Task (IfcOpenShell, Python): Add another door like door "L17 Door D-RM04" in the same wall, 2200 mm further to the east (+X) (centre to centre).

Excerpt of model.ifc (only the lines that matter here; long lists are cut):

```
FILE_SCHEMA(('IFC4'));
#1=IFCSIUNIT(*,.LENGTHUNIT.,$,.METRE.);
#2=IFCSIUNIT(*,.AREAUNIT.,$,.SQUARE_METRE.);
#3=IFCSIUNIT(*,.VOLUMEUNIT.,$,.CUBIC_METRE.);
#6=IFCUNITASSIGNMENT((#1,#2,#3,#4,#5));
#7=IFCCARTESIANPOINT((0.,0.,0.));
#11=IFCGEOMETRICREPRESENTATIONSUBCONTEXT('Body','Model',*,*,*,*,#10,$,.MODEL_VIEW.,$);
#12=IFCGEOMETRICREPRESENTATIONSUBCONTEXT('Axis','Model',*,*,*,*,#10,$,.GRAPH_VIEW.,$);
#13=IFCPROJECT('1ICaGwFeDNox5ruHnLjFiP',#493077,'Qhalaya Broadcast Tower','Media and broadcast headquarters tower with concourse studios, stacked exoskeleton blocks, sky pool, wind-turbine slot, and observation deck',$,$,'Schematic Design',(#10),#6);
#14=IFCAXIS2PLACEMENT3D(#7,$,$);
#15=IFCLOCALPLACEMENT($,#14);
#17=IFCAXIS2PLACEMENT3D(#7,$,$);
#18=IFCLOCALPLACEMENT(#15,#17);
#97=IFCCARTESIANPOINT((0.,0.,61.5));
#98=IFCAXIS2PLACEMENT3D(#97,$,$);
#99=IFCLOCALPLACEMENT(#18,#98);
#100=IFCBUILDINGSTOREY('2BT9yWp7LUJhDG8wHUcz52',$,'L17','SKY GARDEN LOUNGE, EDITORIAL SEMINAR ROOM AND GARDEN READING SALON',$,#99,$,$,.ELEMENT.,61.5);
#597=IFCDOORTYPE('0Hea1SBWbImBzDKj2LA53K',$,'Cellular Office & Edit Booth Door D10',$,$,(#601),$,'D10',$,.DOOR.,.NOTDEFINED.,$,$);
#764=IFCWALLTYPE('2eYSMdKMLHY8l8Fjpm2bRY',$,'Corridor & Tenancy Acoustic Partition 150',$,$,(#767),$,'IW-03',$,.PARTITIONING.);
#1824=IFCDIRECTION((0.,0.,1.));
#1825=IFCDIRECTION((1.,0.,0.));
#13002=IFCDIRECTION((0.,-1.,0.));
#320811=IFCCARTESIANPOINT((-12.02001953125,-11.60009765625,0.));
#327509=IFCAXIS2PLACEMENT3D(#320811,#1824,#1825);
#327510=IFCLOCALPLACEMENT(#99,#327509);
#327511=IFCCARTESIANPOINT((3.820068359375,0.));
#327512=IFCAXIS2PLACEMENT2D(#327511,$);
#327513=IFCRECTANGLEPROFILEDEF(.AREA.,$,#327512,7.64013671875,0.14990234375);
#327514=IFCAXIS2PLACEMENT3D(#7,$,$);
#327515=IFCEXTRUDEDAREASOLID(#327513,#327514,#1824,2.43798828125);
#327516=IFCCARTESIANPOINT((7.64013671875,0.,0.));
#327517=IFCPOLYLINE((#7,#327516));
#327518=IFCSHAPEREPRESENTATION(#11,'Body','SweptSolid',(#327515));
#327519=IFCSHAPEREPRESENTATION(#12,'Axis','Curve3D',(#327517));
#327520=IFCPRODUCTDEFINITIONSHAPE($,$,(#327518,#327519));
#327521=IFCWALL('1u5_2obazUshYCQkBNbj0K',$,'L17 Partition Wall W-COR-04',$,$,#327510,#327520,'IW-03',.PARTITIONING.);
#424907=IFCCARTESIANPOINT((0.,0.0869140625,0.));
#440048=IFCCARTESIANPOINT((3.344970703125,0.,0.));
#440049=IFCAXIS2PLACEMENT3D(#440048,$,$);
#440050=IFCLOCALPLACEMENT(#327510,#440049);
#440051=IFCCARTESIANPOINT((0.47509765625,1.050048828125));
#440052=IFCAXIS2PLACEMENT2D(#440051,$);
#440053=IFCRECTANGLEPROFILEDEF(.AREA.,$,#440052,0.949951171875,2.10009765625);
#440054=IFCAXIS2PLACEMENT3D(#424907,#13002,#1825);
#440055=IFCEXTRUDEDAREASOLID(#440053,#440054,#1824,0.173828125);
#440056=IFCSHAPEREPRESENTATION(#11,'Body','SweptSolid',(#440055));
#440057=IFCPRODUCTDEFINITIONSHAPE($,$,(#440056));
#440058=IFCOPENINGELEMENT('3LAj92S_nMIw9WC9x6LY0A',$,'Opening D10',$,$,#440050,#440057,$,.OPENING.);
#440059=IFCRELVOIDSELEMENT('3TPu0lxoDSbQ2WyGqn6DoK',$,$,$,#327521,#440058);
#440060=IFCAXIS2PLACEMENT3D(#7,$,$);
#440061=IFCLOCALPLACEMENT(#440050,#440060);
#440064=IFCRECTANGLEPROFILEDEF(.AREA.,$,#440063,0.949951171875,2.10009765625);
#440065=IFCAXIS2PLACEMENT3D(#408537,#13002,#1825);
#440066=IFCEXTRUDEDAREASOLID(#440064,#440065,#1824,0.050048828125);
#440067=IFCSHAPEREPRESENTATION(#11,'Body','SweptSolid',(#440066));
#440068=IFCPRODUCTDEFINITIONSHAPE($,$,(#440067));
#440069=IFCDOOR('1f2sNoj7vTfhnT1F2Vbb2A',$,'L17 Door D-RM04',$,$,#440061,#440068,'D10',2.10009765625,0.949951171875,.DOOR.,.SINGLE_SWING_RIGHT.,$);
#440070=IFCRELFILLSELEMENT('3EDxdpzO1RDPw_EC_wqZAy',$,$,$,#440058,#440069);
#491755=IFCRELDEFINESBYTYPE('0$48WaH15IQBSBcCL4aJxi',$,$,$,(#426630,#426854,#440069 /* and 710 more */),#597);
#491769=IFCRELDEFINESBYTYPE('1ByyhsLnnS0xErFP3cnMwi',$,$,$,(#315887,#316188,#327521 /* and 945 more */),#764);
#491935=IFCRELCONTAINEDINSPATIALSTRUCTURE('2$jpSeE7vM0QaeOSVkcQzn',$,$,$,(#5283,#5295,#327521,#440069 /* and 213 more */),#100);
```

```python
import ifcopenshell
import ifcopenshell.api.feature
import ifcopenshell.api.geometry
import ifcopenshell.api.root
import ifcopenshell.geom
import ifcopenshell.util.element
import ifcopenshell.util.placement
import ifcopenshell.util.shape

model = ifcopenshell.open("model.ifc")
settings = ifcopenshell.geom.settings()


def volume(element):
    """Net volume in cubic metres, openings subtracted."""
    shape = ifcopenshell.geom.create_shape(settings, element)
    return ifcopenshell.util.shape.get_volume(shape.geometry)


door = model.by_guid("1f2sNoj7vTfhnT1F2Vbb2A")
opening = door.FillsVoids[0].RelatingOpeningElement
wall = opening.VoidsElements[0].RelatingBuildingElement
before = volume(wall)
shift = ifcopenshell.util.placement.get_local_placement(wall.ObjectPlacement)[:3, 0] * 2.2

# copy_class copies the void relationship, type, container and properties, but no geometry.
new_opening = ifcopenshell.api.root.copy_class(model, product=opening)
new_opening.Representation = ifcopenshell.util.element.copy_deep(
    model, opening.Representation, exclude=["IfcGeometricRepresentationContext", "IfcRepresentationMap"]
)
new_door = ifcopenshell.api.root.copy_class(model, product=door)
new_door.Representation = ifcopenshell.util.element.copy_deep(
    model, door.Representation, exclude=["IfcGeometricRepresentationContext", "IfcRepresentationMap"]
)
new_door.Tag = None
ifcopenshell.api.feature.add_filling(model, opening=new_opening, element=new_door)

for old, new in ((opening, new_opening), (door, new_door)):
    matrix = ifcopenshell.util.placement.get_local_placement(old.ObjectPlacement)
    matrix[:3, 3] += shift
    ifcopenshell.api.geometry.edit_object_placement(model, product=new, matrix=matrix, is_si=False)

after = volume(wall)

print(f"wall volume {before:.3f} -> {after:.3f} m3")

model.write("model_v2.ifc")
```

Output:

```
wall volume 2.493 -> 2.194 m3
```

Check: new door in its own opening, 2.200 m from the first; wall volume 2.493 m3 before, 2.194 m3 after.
